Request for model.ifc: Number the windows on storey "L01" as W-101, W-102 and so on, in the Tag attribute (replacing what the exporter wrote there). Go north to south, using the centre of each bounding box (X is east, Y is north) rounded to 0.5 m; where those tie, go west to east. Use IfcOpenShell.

First a look at what the model holds.

```python
import ifcopenshell
import ifcopenshell.util.element
import ifcopenshell.util.placement

model = ifcopenshell.open("model.ifc")
print(model.schema)
storey = next(s for s in model.by_type("IfcBuildingStorey") if s.Name == "L01")
windows = [e for e in ifcopenshell.util.element.get_decomposition(storey) if e.is_a("IfcWindow")]
for e in sorted(windows, key=lambda e: e.id()):
    origin = ifcopenshell.util.placement.get_local_placement(e.ObjectPlacement)[:3, 3]
    print(e.id(), e.Tag, e.Name, origin.round(2) + 0.0, sep=" | ")
```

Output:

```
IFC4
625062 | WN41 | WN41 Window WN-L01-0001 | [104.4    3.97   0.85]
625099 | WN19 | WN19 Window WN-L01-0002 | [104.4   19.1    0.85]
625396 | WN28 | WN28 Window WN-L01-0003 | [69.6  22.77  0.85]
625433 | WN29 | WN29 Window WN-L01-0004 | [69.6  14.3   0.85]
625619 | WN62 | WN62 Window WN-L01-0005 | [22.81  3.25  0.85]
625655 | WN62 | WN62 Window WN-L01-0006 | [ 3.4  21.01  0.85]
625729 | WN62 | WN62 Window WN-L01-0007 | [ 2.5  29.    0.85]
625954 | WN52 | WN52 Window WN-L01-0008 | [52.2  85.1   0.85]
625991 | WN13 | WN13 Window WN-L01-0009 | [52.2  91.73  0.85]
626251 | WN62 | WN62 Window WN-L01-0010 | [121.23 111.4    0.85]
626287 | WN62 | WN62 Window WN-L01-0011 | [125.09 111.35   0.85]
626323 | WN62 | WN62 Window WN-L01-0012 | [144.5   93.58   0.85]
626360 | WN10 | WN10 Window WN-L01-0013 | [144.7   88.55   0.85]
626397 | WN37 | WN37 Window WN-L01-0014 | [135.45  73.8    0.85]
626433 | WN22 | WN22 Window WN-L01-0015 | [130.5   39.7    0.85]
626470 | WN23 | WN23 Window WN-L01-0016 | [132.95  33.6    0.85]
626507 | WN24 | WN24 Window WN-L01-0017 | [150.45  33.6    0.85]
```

```python
import ifcopenshell
import ifcopenshell.geom
import ifcopenshell.util.element
import ifcopenshell.util.shape

model = ifcopenshell.open("model.ifc")
settings = ifcopenshell.geom.settings()
settings.set("use-world-coords", True)


def centre(element):
    shape = ifcopenshell.geom.create_shape(settings, element)
    return ifcopenshell.util.shape.get_bbox_centroid(shape.geometry)


storey = next(s for s in model.by_type("IfcBuildingStorey") if s.Name == "L01")
windows = [e for e in ifcopenshell.util.element.get_decomposition(storey) if e.is_a("IfcWindow")]

# Insertion points can sit at a corner or the storey origin, so sort by the geometry (in metres).
centres = {e: centre(e) for e in windows}
windows.sort(key=lambda e: (-round(centres[e][1] / 0.5), centres[e][0]))

for i, e in enumerate(windows, start=1):
    number = f"W-1{i:02d}"
    e.Tag = number
    print(e.id(), number)

model.write("model_edited.ifc")
```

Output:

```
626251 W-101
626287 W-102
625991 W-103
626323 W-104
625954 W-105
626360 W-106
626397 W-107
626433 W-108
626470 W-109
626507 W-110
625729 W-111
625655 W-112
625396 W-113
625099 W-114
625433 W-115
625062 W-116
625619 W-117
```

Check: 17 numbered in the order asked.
